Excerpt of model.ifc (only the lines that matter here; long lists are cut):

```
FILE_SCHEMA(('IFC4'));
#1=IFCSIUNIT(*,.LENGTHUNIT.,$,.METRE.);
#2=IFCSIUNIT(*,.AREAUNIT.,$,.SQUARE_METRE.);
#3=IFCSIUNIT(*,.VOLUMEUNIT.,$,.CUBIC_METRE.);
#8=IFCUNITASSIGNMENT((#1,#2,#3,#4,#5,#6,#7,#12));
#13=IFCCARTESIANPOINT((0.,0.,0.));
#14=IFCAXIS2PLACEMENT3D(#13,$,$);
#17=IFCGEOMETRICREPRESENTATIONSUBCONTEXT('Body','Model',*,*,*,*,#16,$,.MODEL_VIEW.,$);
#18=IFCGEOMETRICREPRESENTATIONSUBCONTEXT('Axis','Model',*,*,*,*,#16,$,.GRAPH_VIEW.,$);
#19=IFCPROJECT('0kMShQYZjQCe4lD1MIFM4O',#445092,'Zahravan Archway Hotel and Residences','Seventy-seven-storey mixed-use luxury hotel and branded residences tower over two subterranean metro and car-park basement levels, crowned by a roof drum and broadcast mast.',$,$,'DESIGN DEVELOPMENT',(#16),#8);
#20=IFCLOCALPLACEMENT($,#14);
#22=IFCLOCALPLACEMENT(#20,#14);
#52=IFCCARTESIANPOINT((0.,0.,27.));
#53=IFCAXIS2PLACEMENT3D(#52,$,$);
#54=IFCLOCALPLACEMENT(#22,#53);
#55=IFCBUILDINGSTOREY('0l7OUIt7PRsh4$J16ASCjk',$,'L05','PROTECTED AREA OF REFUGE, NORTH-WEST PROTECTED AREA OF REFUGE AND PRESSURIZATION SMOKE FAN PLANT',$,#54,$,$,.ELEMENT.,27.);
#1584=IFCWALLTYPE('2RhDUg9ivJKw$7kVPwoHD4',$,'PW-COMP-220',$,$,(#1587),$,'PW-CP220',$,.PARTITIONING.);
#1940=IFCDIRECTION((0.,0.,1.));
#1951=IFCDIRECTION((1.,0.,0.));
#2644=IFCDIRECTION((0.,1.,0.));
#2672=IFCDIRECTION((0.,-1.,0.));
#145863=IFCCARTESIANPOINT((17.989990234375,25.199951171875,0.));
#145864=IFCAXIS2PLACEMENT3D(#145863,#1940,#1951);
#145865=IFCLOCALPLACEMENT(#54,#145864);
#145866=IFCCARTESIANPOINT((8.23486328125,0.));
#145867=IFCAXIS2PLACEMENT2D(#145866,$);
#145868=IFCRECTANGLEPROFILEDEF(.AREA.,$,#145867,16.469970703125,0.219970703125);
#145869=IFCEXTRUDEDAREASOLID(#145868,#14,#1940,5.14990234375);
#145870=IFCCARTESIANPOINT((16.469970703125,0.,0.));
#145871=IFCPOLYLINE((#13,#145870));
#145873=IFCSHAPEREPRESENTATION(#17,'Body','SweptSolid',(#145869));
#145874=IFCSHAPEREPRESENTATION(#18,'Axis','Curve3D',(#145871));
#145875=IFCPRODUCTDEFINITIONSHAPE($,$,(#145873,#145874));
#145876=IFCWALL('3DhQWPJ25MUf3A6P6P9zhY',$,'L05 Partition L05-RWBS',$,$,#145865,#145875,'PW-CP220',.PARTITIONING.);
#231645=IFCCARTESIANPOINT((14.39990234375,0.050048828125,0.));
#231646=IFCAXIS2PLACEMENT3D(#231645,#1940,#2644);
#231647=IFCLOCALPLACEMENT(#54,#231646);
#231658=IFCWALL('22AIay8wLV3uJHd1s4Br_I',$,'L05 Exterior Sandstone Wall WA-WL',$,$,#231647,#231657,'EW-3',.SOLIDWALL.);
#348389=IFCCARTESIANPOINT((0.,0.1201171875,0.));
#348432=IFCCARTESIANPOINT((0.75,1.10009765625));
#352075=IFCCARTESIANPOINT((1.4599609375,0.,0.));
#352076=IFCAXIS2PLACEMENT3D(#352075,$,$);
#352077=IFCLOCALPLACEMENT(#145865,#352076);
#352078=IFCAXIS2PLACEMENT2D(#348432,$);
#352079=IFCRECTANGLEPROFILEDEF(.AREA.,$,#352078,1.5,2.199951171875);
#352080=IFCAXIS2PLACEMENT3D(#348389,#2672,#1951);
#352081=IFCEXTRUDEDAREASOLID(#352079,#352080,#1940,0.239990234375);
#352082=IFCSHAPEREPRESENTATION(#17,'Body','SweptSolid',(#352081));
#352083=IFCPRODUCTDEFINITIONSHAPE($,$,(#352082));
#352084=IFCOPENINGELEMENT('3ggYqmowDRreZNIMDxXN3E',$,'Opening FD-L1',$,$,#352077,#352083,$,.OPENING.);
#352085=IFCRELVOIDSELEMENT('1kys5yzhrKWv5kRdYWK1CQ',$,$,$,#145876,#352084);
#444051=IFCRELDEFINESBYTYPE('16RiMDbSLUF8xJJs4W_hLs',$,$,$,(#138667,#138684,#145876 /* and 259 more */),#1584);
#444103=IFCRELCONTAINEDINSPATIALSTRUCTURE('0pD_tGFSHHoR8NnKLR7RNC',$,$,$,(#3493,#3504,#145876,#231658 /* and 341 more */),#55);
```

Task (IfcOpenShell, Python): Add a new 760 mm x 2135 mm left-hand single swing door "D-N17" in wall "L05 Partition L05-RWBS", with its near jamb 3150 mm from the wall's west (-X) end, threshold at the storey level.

```python
import numpy as np
import ifcopenshell
import ifcopenshell.api.feature
import ifcopenshell.api.geometry
import ifcopenshell.api.root
import ifcopenshell.api.spatial
import ifcopenshell.geom
import ifcopenshell.util.element
import ifcopenshell.util.placement
import ifcopenshell.util.representation
import ifcopenshell.util.shape
import ifcopenshell.util.unit

model = ifcopenshell.open("model.ifc")
unit_scale = ifcopenshell.util.unit.calculate_unit_scale(model)
settings = ifcopenshell.geom.settings()


def volume(element):
    """Net volume in cubic metres, openings subtracted."""
    shape = ifcopenshell.geom.create_shape(settings, element)
    return ifcopenshell.util.shape.get_volume(shape.geometry)


wall = model.by_guid("3DhQWPJ25MUf3A6P6P9zhY")
storey = ifcopenshell.util.element.get_container(wall, ifc_class="IfcBuildingStorey")
context = ifcopenshell.util.representation.get_context(model, "Model", "Body", "MODEL_VIEW")
before = volume(wall)

width, height, from_end, sill = 0.76, 2.135, 3.15, 0.0  # metres

# The wall runs along its own X axis, and the end named is its -X end.
wall_shape = ifcopenshell.geom.create_shape(settings, wall)
x, y, z = ifcopenshell.util.shape.get_vertices(wall_shape.geometry).T
start = x.min() + from_end
face, thickness = float(y.min()), float(y.max() - y.min())
wall_matrix = ifcopenshell.util.placement.get_local_placement(wall.ObjectPlacement)
level = ifcopenshell.util.placement.get_local_placement(storey.ObjectPlacement)[2, 3]


def in_wall(x, y):
    """Placement at x, y metres in the wall's axes, at sill height."""
    matrix = wall_matrix.copy()
    matrix[:, 3] = wall_matrix @ np.array([x / unit_scale, y / unit_scale, 0.0, 1.0])
    matrix[2, 3] = level + sill / unit_scale
    return matrix


# Opening: a box that overshoots both wall faces by 50 mm.
opening = ifcopenshell.api.root.create_entity(model, ifc_class="IfcOpeningElement", predefined_type="OPENING")
box = ifcopenshell.api.geometry.add_wall_representation(
    model, context=context, length=width, height=height, thickness=thickness + 0.1
)
ifcopenshell.api.geometry.assign_representation(model, product=opening, representation=box)
ifcopenshell.api.geometry.edit_object_placement(model, product=opening, matrix=in_wall(start, face - 0.05), is_si=False)
ifcopenshell.api.feature.add_feature(model, feature=opening, element=wall)

door = ifcopenshell.api.root.create_entity(model, ifc_class="IfcDoor", name="D-N17", predefined_type="DOOR")
door.OverallWidth, door.OverallHeight = width / unit_scale, height / unit_scale
door.OperationType = "SINGLE_SWING_LEFT"
body = ifcopenshell.api.geometry.add_door_representation(
    model,
    context=context,
    overall_width=door.OverallWidth,
    overall_height=door.OverallHeight,
    operation_type="SINGLE_SWING_LEFT",
    lining_properties={"LiningDepth": thickness / unit_scale, "ThresholdDepth": thickness / unit_scale},
)
ifcopenshell.api.geometry.assign_representation(model, product=door, representation=body)
ifcopenshell.api.spatial.assign_container(model, products=[door], relating_structure=storey)
ifcopenshell.api.feature.add_filling(model, opening=opening, element=door)

# The lining spans the wall, so the door starts at the wall face.
ifcopenshell.api.geometry.edit_object_placement(model, product=door, matrix=in_wall(start, face), is_si=False)

after = volume(wall)

print(f"wall volume {before:.3f} -> {after:.3f} m3")

model.write("model-out.ifc")
```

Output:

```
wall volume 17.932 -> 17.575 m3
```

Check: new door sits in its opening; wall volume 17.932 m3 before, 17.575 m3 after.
